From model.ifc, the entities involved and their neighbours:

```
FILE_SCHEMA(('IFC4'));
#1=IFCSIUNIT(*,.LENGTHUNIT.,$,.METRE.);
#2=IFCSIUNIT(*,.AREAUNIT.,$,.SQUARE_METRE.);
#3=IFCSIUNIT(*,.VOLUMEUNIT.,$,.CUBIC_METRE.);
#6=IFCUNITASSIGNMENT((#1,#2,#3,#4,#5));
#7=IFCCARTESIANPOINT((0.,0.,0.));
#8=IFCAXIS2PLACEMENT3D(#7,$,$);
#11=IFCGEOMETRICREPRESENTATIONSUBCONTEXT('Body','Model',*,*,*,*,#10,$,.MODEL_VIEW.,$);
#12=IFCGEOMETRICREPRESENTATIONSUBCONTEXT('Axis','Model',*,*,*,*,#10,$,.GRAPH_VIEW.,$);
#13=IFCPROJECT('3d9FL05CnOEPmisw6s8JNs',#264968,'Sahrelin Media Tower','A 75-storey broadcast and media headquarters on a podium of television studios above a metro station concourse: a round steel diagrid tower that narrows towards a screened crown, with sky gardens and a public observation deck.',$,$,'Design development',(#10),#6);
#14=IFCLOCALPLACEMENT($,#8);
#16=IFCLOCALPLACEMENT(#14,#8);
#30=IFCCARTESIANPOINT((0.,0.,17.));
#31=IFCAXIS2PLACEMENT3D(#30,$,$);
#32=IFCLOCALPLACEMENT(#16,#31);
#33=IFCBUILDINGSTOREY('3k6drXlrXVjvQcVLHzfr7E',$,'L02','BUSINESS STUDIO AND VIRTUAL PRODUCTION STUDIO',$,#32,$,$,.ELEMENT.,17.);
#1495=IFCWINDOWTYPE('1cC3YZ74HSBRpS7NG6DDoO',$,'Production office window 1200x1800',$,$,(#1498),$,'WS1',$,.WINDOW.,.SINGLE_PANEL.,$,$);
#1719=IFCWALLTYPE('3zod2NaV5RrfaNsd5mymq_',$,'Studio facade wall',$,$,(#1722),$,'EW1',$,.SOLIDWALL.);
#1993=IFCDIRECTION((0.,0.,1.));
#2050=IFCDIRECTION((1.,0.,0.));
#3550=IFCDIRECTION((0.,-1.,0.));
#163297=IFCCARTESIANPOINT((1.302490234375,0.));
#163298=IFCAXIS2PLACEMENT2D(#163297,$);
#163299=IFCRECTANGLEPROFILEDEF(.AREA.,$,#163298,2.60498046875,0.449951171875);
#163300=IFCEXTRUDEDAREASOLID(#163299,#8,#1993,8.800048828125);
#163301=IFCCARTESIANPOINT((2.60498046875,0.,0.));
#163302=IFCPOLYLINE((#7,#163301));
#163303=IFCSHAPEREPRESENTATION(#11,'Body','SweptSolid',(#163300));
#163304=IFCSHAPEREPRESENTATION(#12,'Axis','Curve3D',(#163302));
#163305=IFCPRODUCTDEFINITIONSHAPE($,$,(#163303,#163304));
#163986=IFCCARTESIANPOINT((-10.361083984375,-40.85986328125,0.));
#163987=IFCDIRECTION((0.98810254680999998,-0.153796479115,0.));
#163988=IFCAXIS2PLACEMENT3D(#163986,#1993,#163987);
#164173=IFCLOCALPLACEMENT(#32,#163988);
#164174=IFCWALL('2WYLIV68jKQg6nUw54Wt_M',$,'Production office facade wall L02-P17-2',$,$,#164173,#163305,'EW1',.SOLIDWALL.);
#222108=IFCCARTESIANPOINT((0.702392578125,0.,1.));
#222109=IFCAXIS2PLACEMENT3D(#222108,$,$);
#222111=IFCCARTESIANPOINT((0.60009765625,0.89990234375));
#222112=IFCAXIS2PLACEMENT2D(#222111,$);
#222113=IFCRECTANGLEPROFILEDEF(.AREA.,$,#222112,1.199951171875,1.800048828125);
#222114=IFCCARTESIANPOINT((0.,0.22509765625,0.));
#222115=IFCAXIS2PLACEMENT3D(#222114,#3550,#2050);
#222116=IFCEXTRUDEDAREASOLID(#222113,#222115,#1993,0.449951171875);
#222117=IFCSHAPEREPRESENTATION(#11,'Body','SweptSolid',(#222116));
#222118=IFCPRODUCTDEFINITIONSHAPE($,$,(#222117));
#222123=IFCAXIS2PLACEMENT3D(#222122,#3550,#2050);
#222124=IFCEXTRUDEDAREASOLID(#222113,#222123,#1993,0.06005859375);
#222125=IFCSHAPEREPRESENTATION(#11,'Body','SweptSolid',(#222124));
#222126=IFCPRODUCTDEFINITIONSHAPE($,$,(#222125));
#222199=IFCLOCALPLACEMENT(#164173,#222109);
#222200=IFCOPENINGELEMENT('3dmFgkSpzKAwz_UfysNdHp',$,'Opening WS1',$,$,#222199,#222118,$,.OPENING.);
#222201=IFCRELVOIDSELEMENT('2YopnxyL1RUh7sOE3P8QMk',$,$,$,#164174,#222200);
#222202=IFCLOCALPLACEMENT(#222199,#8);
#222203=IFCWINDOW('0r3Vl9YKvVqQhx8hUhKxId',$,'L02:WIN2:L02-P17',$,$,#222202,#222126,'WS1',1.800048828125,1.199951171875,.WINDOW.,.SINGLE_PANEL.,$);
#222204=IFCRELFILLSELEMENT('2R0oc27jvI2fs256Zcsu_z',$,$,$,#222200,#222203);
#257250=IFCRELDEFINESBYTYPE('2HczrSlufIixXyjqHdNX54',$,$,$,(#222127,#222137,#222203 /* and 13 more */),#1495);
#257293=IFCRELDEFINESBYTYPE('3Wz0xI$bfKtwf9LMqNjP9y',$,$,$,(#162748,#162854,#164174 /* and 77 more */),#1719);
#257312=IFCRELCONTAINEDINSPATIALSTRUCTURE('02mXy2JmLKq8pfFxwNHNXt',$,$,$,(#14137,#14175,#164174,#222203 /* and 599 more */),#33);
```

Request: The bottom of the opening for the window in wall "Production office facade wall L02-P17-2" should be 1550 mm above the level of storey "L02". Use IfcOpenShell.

```python
import numpy as np
import ifcopenshell
import ifcopenshell.api.geometry
import ifcopenshell.geom
import ifcopenshell.util.element
import ifcopenshell.util.placement
import ifcopenshell.util.shape
import ifcopenshell.util.unit

model = ifcopenshell.open("model.ifc")
unit_scale = ifcopenshell.util.unit.calculate_unit_scale(model)

window = model.by_guid("0r3Vl9YKvVqQhx8hUhKxId")
opening = window.FillsVoids[0].RelatingOpeningElement
storey = ifcopenshell.util.element.get_container(window, ifc_class="IfcBuildingStorey")
level = ifcopenshell.util.placement.get_local_placement(storey.ObjectPlacement)[2, 3]

# The opening's origin need not be at the sill, so measure its lowest point.
shape = ifcopenshell.geom.create_shape(ifcopenshell.geom.settings(), opening)
bottom = ifcopenshell.util.shape.get_shape_bottom_elevation(shape, shape.geometry) / unit_scale
dz = level + 1.55 / unit_scale - bottom

shift = np.array([0.0, 0.0, dz])
# The window is placed relative to its opening, so it follows when the opening moves.
matrix = ifcopenshell.util.placement.get_local_placement(opening.ObjectPlacement)
matrix[:3, 3] += shift
ifcopenshell.api.geometry.edit_object_placement(
    model, product=opening, matrix=matrix, is_si=False, should_transform_children=True
)

print(f"moved by {dz * unit_scale:+.3f} m")

model.write("model_rev.ifc")
```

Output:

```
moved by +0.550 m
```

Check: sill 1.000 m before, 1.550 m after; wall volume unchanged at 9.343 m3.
